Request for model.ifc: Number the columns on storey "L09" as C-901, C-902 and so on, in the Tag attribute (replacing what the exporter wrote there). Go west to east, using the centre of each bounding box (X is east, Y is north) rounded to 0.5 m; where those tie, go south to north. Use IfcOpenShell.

First a look at what the model holds.

```python
import ifcopenshell
import ifcopenshell.util.element
import ifcopenshell.util.placement

model = ifcopenshell.open("model.ifc")
print(model.schema)
storey = next(s for s in model.by_type("IfcBuildingStorey") if s.Name == "L09")
columns = [e for e in ifcopenshell.util.element.get_decomposition(storey) if e.is_a("IfcColumn")]
for e in sorted(columns, key=lambda e: e.id()):
    origin = ifcopenshell.util.placement.get_local_placement(e.ObjectPlacement)[:3, 3]
    print(e.id(), e.Tag, e.Name, origin.round(2) + 0.0, sep=" | ")
```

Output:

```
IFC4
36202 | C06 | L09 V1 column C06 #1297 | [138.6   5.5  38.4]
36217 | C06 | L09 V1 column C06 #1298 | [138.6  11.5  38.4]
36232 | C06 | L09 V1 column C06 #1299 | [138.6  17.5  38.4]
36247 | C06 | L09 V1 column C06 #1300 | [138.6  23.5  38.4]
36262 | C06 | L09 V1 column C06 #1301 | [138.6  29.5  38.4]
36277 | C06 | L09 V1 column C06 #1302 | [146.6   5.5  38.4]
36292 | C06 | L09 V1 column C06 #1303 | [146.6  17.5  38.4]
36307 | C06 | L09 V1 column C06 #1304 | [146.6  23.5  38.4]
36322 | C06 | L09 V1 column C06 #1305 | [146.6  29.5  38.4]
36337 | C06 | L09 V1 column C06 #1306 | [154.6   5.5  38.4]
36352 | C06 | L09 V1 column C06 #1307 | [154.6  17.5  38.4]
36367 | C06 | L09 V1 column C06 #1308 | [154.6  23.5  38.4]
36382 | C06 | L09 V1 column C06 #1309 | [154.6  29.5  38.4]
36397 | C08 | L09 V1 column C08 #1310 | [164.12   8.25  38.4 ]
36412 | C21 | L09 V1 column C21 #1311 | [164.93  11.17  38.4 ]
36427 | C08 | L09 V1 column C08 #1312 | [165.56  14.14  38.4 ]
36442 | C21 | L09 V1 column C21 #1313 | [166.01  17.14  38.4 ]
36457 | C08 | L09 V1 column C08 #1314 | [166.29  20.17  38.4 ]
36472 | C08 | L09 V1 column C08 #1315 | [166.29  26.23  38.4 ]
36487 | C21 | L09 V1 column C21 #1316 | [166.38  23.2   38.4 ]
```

```python
import ifcopenshell
import ifcopenshell.geom
import ifcopenshell.util.element
import ifcopenshell.util.shape

model = ifcopenshell.open("model.ifc")
settings = ifcopenshell.geom.settings()
settings.set("use-world-coords", True)


def centre(element):
    shape = ifcopenshell.geom.create_shape(settings, element)
    return ifcopenshell.util.shape.get_bbox_centroid(shape.geometry)


storey = next(s for s in model.by_type("IfcBuildingStorey") if s.Name == "L09")
columns = [e for e in ifcopenshell.util.element.get_decomposition(storey) if e.is_a("IfcColumn")]

# Insertion points can sit at a corner or the storey origin, so sort by the geometry (in metres).
centres = {e: centre(e) for e in columns}
columns.sort(key=lambda e: (round(centres[e][0] / 0.5), centres[e][1]))

for i, e in enumerate(columns, start=1):
    number = f"C-9{i:02d}"
    e.Tag = number
    print(e.id(), number)

model.write("model_rev.ifc")
```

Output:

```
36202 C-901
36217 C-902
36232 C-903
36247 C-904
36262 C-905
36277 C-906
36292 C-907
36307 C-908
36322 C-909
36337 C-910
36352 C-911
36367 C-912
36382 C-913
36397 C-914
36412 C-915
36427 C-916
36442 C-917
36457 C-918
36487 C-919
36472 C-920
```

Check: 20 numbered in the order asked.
